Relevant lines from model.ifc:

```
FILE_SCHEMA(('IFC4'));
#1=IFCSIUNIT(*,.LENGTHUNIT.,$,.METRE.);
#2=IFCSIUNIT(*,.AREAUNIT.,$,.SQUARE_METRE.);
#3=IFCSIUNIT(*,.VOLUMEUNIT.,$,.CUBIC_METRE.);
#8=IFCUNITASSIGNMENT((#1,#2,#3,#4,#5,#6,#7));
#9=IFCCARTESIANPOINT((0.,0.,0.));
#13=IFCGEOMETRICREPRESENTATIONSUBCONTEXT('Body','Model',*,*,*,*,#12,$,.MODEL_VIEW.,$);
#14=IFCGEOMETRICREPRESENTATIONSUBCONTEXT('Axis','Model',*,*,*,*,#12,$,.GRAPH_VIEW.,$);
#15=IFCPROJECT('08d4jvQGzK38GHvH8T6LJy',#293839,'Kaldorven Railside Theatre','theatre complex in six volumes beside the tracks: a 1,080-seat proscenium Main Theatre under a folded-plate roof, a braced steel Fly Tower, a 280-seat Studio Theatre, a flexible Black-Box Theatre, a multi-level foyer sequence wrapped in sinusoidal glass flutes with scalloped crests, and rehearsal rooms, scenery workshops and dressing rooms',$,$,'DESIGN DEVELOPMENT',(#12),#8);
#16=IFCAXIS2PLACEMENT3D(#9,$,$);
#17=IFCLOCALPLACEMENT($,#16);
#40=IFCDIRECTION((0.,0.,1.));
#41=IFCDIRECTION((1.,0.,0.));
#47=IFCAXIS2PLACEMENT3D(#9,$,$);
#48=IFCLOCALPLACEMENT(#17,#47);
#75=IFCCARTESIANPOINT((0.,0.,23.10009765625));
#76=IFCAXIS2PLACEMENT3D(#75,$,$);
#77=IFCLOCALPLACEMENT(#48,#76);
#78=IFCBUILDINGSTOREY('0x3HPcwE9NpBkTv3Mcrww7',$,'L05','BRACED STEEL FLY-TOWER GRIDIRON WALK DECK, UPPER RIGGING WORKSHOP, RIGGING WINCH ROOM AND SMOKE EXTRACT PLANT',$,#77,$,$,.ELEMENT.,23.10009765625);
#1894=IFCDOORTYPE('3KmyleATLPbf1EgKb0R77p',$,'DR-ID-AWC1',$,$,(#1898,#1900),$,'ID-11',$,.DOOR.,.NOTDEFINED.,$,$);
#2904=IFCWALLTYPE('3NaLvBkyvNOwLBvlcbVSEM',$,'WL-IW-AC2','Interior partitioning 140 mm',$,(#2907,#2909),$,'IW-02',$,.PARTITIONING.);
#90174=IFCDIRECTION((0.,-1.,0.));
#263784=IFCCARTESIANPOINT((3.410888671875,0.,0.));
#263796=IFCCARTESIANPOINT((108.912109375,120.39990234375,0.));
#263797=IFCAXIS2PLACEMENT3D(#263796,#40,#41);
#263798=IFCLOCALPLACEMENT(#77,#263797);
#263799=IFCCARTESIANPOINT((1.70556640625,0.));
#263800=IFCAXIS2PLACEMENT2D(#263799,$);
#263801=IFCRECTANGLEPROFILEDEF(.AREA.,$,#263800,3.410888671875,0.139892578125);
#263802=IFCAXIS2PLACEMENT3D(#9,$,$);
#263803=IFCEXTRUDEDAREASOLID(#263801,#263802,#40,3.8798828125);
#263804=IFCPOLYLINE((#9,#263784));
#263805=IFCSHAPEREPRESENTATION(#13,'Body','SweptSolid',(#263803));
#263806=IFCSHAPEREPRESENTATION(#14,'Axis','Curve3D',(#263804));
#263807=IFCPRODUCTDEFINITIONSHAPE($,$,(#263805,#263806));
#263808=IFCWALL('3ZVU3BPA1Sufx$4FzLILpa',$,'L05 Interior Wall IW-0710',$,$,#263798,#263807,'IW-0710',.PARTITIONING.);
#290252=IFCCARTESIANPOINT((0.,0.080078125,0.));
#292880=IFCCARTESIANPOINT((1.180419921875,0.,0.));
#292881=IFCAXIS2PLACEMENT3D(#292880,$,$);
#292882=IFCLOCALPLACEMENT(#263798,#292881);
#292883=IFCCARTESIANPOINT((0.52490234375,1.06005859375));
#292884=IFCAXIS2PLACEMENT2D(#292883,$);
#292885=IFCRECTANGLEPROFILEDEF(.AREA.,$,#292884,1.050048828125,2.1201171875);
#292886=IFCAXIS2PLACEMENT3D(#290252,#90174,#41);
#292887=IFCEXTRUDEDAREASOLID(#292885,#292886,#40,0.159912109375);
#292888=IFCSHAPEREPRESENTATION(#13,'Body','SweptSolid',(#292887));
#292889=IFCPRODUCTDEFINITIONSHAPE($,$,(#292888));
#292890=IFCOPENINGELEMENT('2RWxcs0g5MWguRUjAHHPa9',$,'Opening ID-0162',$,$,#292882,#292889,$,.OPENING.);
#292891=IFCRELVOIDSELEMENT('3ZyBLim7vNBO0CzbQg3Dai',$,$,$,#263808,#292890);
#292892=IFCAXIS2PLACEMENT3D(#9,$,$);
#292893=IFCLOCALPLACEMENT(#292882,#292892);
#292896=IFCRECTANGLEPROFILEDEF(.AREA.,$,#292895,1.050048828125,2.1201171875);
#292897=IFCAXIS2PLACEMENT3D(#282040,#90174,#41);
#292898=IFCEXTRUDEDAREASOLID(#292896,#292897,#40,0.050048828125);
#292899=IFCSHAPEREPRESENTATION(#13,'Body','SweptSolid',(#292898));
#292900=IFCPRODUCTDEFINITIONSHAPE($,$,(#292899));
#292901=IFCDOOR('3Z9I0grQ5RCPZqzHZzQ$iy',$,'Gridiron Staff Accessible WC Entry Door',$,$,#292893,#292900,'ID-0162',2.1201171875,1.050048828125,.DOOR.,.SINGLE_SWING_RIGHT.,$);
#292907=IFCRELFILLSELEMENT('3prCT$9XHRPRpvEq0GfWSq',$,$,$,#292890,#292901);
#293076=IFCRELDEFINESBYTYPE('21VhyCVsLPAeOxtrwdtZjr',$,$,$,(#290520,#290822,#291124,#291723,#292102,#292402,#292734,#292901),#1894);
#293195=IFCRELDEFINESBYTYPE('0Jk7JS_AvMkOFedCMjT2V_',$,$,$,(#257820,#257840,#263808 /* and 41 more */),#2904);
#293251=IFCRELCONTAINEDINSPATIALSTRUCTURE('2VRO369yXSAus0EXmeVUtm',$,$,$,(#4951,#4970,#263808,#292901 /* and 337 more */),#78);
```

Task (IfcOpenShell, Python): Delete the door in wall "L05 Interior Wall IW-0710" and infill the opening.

```python
import ifcopenshell
import ifcopenshell.api.feature
import ifcopenshell.api.root
import ifcopenshell.geom
import ifcopenshell.util.shape

model = ifcopenshell.open("model.ifc")
settings = ifcopenshell.geom.settings()


def volume(element):
    """Net volume in cubic metres, openings subtracted."""
    shape = ifcopenshell.geom.create_shape(settings, element)
    return ifcopenshell.util.shape.get_volume(shape.geometry)


door = model.by_guid("3Z9I0grQ5RCPZqzHZzQ$iy")
opening = door.FillsVoids[0].RelatingOpeningElement
wall = opening.VoidsElements[0].RelatingBuildingElement
before = volume(wall)

ifcopenshell.api.root.remove_product(model, product=door)
ifcopenshell.api.feature.remove_feature(model, feature=opening)

after = volume(wall)

print(f"wall volume {before:.3f} -> {after:.3f} m3")

model.write("model-out.ifc")
```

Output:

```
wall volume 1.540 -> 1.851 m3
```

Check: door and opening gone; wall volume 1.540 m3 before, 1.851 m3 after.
